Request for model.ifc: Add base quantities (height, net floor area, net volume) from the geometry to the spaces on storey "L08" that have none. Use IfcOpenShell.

First a look at what the model holds.

```python
import ifcopenshell
import ifcopenshell.util.element
import ifcopenshell.util.unit

model = ifcopenshell.open("model.ifc")
print(model.schema)
for unit_type in ("LENGTHUNIT", "AREAUNIT", "VOLUMEUNIT"):
    print(unit_type, ifcopenshell.util.unit.calculate_unit_scale(model, unit_type))
storey = next(s for s in model.by_type("IfcBuildingStorey") if s.Name == "L08")
spaces = [e for e in ifcopenshell.util.element.get_decomposition(storey) if e.is_a("IfcSpace")]
for e in sorted(spaces, key=lambda e: e.id()):
    print(e.id(), e.is_a(), e.Name, list(ifcopenshell.util.element.get_psets(e, qtos_only=True)), sep=" | ")
```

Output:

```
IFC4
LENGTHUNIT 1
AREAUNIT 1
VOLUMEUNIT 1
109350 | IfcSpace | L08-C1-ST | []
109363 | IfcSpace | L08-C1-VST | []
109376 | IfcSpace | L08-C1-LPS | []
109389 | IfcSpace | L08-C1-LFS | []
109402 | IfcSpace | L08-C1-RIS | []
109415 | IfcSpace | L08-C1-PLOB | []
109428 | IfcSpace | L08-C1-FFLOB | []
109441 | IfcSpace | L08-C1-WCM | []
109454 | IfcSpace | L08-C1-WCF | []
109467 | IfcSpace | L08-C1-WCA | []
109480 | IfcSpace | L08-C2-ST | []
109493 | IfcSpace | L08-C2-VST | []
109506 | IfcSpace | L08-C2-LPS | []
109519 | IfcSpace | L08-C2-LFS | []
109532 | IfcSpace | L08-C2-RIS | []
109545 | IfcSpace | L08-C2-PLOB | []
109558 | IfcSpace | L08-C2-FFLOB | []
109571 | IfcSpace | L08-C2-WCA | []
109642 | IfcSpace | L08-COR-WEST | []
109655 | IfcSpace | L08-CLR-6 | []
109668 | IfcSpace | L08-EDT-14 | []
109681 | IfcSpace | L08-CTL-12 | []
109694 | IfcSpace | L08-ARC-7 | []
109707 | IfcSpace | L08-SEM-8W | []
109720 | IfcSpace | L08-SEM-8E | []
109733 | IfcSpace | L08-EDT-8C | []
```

```python
import ifcopenshell
import ifcopenshell.api.pset
import ifcopenshell.geom
import ifcopenshell.util.element
import ifcopenshell.util.shape
import ifcopenshell.util.unit

model = ifcopenshell.open("model.ifc")
unit_scale = ifcopenshell.util.unit.calculate_unit_scale(model)
area_scale = ifcopenshell.util.unit.calculate_unit_scale(model, "AREAUNIT")
volume_scale = ifcopenshell.util.unit.calculate_unit_scale(model, "VOLUMEUNIT")
settings = ifcopenshell.geom.settings()

storey = next(s for s in model.by_type("IfcBuildingStorey") if s.Name == "L08")
spaces = [e for e in ifcopenshell.util.element.get_decomposition(storey) if e.is_a("IfcSpace")]

for e in sorted(spaces, key=lambda e: e.id()):
    if ifcopenshell.util.element.get_psets(e, qtos_only=True, should_inherit=False):
        continue
    # Geometry comes back in metres, in the element's own axes.
    shape = ifcopenshell.geom.create_shape(settings, e)
    values = {
        "Height": ifcopenshell.util.shape.get_z(shape.geometry) / unit_scale,
        "NetFloorArea": ifcopenshell.util.shape.get_footprint_area(shape.geometry) / area_scale,
        "NetVolume": ifcopenshell.util.shape.get_volume(shape.geometry) / volume_scale,
    }
    qto = ifcopenshell.api.pset.add_qto(model, product=e, name="Qto_SpaceBaseQuantities")
    ifcopenshell.api.pset.edit_qto(model, qto=qto, properties=values)
    print(e.id(), {k: round(v, 3) for k, v in values.items()})

model.write("model_v2.ifc")
```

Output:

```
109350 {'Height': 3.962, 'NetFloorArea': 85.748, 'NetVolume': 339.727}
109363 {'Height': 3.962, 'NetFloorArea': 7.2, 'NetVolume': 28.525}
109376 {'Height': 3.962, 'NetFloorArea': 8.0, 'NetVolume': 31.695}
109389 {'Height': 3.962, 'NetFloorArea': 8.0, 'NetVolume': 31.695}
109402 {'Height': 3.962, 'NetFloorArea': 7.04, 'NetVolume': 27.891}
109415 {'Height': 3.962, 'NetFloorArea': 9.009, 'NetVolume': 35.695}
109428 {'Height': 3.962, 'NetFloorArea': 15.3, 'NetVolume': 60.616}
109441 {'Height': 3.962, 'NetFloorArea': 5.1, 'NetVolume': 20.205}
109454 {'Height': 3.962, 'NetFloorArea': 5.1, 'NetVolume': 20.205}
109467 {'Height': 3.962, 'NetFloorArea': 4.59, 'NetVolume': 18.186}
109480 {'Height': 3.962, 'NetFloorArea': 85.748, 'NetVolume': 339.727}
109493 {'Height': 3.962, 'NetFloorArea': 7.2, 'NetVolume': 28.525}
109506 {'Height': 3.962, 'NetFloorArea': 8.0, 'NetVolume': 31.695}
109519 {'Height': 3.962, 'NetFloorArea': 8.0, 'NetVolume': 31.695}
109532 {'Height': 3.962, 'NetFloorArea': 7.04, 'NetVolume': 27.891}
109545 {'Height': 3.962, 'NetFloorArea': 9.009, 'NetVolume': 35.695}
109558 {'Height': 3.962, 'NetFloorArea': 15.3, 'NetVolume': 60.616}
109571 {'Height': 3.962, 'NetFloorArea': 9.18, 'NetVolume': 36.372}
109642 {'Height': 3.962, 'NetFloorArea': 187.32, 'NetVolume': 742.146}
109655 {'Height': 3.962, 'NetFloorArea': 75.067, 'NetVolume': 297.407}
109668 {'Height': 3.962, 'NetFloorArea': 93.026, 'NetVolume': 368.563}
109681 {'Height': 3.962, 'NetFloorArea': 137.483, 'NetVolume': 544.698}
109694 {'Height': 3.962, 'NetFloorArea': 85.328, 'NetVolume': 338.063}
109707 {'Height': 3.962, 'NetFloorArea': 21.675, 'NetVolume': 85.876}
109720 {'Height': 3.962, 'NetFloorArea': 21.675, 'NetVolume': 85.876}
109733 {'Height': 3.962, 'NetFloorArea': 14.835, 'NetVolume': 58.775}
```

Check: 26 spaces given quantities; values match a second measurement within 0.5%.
